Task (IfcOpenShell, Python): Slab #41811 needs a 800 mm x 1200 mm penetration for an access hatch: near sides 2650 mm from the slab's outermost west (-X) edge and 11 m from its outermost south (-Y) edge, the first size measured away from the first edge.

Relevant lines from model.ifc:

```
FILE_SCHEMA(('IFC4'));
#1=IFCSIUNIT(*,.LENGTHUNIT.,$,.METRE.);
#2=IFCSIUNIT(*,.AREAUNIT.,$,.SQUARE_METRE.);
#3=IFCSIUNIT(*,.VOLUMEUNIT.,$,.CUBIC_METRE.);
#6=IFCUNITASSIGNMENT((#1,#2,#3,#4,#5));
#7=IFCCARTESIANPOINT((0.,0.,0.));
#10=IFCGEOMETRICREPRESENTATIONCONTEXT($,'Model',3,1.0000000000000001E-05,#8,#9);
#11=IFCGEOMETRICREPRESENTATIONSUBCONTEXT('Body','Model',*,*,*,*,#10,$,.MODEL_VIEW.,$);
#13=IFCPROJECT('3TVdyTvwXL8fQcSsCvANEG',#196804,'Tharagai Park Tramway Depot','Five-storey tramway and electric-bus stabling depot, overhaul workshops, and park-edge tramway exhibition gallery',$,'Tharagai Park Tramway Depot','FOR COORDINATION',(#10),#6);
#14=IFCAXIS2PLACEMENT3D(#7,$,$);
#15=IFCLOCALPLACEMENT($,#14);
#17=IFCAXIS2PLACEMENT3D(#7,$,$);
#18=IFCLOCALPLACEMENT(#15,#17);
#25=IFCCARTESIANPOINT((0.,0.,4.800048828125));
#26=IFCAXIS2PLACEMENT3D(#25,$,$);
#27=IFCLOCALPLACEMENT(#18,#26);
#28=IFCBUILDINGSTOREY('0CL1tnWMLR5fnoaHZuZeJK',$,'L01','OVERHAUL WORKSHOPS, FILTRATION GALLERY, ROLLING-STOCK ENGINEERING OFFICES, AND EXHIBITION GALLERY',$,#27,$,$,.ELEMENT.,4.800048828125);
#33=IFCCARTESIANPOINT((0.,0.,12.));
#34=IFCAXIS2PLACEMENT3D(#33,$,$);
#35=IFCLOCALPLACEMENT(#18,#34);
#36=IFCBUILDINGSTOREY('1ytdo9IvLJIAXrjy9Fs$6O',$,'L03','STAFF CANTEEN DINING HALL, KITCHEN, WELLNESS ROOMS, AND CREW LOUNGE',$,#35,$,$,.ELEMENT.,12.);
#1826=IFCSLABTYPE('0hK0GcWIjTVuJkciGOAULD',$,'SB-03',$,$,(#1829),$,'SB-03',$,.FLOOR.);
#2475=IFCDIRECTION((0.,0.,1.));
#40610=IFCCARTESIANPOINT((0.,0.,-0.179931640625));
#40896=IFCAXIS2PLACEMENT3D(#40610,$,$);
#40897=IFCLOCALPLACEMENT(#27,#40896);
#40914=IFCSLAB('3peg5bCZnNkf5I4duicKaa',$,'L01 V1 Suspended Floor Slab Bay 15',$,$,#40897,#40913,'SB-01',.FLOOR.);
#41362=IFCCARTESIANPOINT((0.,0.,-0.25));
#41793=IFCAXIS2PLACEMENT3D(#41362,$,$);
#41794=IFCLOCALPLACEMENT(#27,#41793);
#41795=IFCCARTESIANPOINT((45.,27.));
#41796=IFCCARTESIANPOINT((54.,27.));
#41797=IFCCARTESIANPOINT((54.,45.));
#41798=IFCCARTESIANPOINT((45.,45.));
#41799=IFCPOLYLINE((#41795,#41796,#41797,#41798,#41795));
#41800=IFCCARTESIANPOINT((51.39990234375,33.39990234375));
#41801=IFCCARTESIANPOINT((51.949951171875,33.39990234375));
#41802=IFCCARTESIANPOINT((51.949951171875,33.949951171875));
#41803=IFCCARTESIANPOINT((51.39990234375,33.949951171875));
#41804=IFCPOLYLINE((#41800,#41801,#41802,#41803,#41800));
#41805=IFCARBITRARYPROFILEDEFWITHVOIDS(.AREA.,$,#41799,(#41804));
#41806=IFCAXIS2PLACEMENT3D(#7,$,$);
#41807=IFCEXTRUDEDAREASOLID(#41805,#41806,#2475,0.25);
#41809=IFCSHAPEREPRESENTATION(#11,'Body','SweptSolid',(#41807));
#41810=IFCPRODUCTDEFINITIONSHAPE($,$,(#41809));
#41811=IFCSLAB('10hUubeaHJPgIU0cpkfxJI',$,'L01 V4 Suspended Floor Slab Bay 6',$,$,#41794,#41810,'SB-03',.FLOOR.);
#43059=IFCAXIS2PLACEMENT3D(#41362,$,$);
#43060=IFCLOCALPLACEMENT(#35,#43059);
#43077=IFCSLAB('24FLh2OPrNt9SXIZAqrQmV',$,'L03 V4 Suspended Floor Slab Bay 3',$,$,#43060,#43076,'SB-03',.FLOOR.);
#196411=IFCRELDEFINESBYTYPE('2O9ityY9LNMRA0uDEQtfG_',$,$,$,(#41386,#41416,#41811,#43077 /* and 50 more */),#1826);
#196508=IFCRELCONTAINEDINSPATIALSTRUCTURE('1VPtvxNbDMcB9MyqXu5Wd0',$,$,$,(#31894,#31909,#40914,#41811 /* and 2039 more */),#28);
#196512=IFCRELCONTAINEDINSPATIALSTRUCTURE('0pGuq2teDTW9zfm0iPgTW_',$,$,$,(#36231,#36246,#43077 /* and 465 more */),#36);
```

```python
import numpy as np
import ifcopenshell
import ifcopenshell.api.feature
import ifcopenshell.api.geometry
import ifcopenshell.api.root
import ifcopenshell.geom
import ifcopenshell.util.placement
import ifcopenshell.util.representation
import ifcopenshell.util.shape
import ifcopenshell.util.unit

model = ifcopenshell.open("model.ifc")
unit_scale = ifcopenshell.util.unit.calculate_unit_scale(model)
settings = ifcopenshell.geom.settings()


def volume(element):
    """Net volume in cubic metres, openings subtracted."""
    shape = ifcopenshell.geom.create_shape(settings, element)
    return ifcopenshell.util.shape.get_volume(shape.geometry)


slab = model.by_guid("10hUubeaHJPgIU0cpkfxJI")
before = volume(slab)

# Extent in the slab's own axes, in metres. The edges named are its -X and -Y sides.
slab_shape = ifcopenshell.geom.create_shape(settings, slab)
vertices = ifcopenshell.util.shape.get_vertices(slab_shape.geometry)
x_min, y_min, bottom = vertices.min(axis=0)
top = vertices[:, 2].max()

opening = ifcopenshell.api.root.create_entity(model, ifc_class="IfcOpeningElement", name="Access hatch opening", predefined_type="OPENING")
context = ifcopenshell.util.representation.get_context(model, "Model", "Body", "MODEL_VIEW")
width, depth = 0.8, 1.2
outline = [(0.0, 0.0), (width, 0.0), (width, depth), (0.0, depth), (0.0, 0.0)]
# Overshoot both faces by 50 mm so the cut is clean.
shape = ifcopenshell.api.geometry.add_slab_representation(
    model, context=context, depth=top - bottom + 0.1, polyline=outline
)
ifcopenshell.api.geometry.assign_representation(model, product=opening, representation=shape)

matrix = ifcopenshell.util.placement.get_local_placement(slab.ObjectPlacement)
matrix[:, 3] = matrix @ np.append(np.array([x_min + 2.65, y_min + 11, bottom - 0.05]) / unit_scale, 1.0)
ifcopenshell.api.geometry.edit_object_placement(model, product=opening, matrix=matrix, is_si=False)
ifcopenshell.api.feature.add_feature(model, feature=opening, element=slab)

after = volume(slab)

print(f"slab volume {before:.3f} -> {after:.3f} m3")

model.write("model_v2.ifc")
```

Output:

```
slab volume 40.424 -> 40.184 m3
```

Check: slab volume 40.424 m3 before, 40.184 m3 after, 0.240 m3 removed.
